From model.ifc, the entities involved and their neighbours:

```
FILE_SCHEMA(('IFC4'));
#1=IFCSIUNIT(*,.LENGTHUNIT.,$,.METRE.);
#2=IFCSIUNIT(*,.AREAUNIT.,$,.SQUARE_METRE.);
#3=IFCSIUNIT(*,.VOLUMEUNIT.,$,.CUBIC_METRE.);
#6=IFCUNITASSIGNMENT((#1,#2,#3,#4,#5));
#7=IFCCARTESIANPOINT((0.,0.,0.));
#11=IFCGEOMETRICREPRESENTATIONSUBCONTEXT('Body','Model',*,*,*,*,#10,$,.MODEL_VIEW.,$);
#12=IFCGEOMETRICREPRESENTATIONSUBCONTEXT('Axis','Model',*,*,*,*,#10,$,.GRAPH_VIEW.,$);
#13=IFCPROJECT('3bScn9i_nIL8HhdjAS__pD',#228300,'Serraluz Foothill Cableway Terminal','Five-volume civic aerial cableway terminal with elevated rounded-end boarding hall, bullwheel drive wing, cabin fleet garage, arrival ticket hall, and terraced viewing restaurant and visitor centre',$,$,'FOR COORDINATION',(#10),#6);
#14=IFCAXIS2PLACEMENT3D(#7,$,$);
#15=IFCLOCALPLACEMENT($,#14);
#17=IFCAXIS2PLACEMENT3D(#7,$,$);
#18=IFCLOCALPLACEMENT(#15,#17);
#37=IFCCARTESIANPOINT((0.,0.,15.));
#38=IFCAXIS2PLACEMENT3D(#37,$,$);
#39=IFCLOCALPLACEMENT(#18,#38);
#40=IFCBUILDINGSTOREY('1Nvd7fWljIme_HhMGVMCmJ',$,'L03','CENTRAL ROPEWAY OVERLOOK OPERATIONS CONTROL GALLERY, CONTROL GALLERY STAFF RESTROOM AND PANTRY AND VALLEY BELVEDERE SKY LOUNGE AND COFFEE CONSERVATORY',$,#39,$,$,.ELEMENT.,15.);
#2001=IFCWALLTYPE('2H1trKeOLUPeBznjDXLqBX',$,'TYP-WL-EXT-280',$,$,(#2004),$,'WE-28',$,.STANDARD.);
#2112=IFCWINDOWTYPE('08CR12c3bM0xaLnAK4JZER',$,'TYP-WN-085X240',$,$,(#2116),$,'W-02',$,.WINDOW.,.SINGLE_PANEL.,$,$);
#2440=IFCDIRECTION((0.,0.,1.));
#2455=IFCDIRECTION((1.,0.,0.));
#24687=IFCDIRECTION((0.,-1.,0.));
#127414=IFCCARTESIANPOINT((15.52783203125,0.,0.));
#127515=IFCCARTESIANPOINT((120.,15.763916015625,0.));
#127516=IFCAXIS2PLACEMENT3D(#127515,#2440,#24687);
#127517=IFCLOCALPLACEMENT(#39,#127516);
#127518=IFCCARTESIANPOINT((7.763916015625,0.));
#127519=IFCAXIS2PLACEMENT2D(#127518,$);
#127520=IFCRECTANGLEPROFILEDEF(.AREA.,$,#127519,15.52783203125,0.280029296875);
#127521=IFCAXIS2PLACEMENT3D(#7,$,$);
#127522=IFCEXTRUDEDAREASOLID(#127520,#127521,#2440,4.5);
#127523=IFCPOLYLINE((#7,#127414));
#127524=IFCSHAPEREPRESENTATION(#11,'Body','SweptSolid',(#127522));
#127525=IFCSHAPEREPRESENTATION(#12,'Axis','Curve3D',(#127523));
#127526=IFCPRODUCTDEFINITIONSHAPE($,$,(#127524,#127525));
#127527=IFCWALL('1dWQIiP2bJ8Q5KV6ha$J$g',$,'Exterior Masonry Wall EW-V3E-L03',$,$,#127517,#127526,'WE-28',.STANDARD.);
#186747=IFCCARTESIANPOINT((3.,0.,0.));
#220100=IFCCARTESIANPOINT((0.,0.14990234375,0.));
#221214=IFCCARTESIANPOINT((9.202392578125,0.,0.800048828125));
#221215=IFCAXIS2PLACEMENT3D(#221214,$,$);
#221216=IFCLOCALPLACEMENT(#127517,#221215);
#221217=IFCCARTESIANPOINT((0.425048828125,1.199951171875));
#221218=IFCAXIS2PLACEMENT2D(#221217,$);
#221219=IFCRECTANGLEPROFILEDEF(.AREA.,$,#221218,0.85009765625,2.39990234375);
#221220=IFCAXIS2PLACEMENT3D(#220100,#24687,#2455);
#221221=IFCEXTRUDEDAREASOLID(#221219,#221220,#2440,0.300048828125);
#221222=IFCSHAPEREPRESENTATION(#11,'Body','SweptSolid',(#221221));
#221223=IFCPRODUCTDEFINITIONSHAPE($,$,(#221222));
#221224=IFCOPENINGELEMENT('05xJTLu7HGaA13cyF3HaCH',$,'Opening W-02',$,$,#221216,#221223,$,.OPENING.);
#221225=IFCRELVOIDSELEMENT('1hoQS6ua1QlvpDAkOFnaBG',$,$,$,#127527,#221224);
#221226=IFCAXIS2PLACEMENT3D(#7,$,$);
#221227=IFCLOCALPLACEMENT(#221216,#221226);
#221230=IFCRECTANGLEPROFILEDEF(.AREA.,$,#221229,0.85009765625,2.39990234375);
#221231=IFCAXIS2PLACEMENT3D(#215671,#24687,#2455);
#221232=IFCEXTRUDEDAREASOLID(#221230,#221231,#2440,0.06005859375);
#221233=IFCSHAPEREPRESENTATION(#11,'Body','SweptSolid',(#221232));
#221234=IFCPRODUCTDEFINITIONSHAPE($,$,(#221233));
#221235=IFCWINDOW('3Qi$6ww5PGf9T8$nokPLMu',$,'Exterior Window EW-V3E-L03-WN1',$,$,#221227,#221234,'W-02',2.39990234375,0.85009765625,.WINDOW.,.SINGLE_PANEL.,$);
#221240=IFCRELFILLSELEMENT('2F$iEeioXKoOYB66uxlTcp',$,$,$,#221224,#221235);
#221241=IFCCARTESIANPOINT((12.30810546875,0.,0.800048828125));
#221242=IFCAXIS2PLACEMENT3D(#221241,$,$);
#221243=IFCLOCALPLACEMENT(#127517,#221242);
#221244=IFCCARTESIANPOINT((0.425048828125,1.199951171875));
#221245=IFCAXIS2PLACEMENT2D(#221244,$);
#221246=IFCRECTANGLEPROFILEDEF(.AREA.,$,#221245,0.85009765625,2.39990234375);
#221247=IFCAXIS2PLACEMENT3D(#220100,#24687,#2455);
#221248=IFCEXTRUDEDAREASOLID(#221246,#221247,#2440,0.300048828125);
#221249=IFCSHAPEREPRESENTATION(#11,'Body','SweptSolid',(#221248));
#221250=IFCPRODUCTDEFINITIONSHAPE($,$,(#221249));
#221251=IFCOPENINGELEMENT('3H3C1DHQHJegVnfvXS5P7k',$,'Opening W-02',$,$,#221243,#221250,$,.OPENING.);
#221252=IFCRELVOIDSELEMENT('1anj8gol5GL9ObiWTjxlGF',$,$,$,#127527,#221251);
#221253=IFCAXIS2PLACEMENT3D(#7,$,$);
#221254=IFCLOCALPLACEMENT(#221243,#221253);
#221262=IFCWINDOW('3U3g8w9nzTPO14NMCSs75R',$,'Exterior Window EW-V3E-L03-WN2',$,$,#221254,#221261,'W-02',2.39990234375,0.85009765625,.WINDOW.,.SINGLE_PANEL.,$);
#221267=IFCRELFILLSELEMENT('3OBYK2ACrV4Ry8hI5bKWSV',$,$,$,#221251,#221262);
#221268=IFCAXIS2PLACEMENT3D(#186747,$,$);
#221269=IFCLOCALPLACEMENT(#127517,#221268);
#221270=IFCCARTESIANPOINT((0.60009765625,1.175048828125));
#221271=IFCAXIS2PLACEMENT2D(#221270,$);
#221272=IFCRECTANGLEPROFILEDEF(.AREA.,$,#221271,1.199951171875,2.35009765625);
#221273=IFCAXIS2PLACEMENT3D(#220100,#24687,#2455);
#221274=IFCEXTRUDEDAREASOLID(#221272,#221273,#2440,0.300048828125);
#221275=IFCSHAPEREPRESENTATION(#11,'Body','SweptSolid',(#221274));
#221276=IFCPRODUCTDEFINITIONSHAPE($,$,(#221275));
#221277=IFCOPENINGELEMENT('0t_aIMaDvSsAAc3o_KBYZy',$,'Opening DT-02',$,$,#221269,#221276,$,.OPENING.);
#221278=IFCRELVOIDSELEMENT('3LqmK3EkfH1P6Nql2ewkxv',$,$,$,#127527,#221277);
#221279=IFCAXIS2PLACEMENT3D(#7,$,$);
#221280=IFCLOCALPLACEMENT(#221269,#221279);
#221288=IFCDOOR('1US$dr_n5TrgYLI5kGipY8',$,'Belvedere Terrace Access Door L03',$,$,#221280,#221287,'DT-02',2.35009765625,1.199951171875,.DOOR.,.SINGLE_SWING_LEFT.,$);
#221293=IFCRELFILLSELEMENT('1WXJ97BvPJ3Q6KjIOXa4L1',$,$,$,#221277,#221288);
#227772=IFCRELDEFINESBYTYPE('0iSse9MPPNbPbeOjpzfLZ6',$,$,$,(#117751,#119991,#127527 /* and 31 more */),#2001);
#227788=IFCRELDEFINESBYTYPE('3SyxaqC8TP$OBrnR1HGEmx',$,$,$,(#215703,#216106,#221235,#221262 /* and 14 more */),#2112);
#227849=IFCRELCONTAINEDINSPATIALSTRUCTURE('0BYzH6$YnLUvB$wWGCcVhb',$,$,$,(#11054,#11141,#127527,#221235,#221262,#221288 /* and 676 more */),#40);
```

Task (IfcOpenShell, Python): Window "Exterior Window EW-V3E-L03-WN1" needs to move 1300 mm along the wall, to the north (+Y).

```python
import ifcopenshell
import ifcopenshell.api.geometry
import ifcopenshell.util.placement
import ifcopenshell.util.unit

model = ifcopenshell.open("model.ifc")
unit_scale = ifcopenshell.util.unit.calculate_unit_scale(model)

window = model.by_id(221235)
opening = window.FillsVoids[0].RelatingOpeningElement
wall = opening.VoidsElements[0].RelatingBuildingElement

wall_matrix = ifcopenshell.util.placement.get_local_placement(wall.ObjectPlacement)
shift = wall_matrix[:3, 0] * -1.3 / unit_scale
before = ifcopenshell.util.placement.get_local_placement(window.ObjectPlacement)[:3, 3].copy()

# The window is placed relative to its opening, so it follows when the opening moves.
matrix = ifcopenshell.util.placement.get_local_placement(opening.ObjectPlacement)
matrix[:3, 3] += shift
ifcopenshell.api.geometry.edit_object_placement(
    model, product=opening, matrix=matrix, is_si=False, should_transform_children=True
)

after = ifcopenshell.util.placement.get_local_placement(window.ObjectPlacement)[:3, 3]
print("window moved by", (after - before).round(3) + 0.0)

model.write("model_edited.ifc")
```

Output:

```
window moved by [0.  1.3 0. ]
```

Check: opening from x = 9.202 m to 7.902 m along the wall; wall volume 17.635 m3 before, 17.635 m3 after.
